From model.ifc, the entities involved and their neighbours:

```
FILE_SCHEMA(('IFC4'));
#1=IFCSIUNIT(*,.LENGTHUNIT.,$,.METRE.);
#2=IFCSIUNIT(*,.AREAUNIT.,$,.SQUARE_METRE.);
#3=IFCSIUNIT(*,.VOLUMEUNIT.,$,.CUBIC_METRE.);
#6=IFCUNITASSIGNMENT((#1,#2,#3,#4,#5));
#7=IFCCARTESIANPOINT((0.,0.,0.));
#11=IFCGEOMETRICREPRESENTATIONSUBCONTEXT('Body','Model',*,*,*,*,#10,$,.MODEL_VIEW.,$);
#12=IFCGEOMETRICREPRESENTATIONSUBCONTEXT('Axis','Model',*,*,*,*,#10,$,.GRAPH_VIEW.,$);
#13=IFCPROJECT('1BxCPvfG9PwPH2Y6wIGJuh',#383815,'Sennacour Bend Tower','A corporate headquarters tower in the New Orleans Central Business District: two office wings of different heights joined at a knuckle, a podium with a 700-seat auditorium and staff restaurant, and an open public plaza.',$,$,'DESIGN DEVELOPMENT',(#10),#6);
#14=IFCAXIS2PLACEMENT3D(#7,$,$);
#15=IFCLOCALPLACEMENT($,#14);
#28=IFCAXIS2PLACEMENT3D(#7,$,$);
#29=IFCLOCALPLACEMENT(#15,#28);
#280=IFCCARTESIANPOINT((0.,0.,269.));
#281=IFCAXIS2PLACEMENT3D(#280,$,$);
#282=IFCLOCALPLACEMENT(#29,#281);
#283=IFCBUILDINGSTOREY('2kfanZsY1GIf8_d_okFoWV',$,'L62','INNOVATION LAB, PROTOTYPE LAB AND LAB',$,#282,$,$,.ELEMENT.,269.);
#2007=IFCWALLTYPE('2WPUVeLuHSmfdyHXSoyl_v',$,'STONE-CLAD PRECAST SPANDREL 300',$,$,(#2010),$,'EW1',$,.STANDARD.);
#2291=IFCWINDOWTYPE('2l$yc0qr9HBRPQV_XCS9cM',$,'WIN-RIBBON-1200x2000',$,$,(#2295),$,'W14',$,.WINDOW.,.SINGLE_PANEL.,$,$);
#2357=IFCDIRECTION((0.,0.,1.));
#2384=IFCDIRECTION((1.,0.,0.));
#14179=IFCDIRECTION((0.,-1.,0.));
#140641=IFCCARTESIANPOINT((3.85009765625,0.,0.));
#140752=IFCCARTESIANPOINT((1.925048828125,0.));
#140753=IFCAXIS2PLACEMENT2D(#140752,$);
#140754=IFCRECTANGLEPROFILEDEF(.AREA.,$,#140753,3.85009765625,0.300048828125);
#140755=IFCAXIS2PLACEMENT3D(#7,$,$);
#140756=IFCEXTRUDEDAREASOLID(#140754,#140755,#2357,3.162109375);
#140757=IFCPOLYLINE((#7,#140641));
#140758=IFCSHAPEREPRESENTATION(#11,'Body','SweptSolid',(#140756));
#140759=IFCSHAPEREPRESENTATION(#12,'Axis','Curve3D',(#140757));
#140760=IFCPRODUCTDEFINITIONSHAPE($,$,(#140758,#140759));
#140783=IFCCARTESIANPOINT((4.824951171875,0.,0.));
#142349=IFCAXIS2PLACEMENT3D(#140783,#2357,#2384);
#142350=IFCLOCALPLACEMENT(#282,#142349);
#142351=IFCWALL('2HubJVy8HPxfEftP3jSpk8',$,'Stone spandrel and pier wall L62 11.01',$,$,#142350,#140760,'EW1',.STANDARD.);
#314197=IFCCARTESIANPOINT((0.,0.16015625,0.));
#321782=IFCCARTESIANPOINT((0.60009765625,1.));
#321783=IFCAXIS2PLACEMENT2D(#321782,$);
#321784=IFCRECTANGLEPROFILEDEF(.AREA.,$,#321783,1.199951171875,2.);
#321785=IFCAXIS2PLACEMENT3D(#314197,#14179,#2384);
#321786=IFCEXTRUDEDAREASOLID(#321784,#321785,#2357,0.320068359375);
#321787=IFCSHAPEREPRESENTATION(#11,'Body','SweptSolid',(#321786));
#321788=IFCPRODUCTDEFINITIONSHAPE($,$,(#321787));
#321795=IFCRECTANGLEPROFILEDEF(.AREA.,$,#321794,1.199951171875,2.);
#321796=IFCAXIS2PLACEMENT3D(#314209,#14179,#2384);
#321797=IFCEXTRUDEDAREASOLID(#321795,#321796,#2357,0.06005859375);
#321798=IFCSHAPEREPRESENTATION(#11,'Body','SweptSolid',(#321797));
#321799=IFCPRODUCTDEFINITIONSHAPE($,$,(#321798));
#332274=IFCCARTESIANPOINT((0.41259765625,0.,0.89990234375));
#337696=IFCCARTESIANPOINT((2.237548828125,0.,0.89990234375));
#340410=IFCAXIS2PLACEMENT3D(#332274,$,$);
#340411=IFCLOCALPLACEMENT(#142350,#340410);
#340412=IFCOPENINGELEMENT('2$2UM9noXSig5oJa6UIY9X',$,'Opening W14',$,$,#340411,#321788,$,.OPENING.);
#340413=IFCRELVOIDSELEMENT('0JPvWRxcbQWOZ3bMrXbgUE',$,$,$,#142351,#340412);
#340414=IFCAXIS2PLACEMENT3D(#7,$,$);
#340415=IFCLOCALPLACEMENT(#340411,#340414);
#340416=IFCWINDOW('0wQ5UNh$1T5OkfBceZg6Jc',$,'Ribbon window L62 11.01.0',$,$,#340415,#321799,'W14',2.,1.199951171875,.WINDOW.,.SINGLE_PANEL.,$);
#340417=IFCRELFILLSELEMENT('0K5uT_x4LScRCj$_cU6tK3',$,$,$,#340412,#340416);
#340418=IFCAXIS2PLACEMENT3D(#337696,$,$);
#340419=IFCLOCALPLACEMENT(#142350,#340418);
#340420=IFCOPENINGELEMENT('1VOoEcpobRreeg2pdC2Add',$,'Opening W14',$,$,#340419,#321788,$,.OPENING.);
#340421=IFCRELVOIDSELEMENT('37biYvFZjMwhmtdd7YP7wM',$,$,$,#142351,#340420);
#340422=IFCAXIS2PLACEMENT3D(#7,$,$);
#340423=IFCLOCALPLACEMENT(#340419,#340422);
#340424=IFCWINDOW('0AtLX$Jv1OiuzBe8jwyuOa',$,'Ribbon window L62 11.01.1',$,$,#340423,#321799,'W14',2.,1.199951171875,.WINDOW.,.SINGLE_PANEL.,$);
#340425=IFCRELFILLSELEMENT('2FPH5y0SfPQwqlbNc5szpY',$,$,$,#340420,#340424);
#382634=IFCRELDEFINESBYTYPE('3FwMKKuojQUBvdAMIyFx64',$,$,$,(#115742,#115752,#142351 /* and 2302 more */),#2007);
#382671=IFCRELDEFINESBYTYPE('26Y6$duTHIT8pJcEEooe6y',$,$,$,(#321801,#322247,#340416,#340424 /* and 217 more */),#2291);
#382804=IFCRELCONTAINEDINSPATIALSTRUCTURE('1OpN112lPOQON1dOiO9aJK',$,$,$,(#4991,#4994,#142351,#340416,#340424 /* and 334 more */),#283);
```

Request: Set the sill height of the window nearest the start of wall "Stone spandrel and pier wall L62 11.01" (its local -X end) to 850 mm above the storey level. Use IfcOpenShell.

```python
import numpy as np
import ifcopenshell
import ifcopenshell.api.geometry
import ifcopenshell.geom
import ifcopenshell.util.element
import ifcopenshell.util.placement
import ifcopenshell.util.shape
import ifcopenshell.util.unit

model = ifcopenshell.open("model.ifc")
unit_scale = ifcopenshell.util.unit.calculate_unit_scale(model)

window = model.by_guid("0wQ5UNh$1T5OkfBceZg6Jc")
opening = window.FillsVoids[0].RelatingOpeningElement
storey = ifcopenshell.util.element.get_container(window, ifc_class="IfcBuildingStorey")
level = ifcopenshell.util.placement.get_local_placement(storey.ObjectPlacement)[2, 3]

# The opening's origin need not be at the sill, so measure its lowest point.
shape = ifcopenshell.geom.create_shape(ifcopenshell.geom.settings(), opening)
bottom = ifcopenshell.util.shape.get_shape_bottom_elevation(shape, shape.geometry) / unit_scale
dz = level + 0.85 / unit_scale - bottom

shift = np.array([0.0, 0.0, dz])
# The window is placed relative to its opening, so it follows when the opening moves.
matrix = ifcopenshell.util.placement.get_local_placement(opening.ObjectPlacement)
matrix[:3, 3] += shift
ifcopenshell.api.geometry.edit_object_placement(
    model, product=opening, matrix=matrix, is_si=False, should_transform_children=True
)

print(f"moved by {dz * unit_scale:+.3f} m")

model.write("model_updated.ifc")
```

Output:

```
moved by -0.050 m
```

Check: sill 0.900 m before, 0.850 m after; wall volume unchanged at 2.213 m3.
